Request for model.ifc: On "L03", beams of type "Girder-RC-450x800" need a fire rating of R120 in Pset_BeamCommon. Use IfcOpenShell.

First a look at what the model holds.

```python
import ifcopenshell
import ifcopenshell.util.element

model = ifcopenshell.open("model.ifc")
print(model.schema)
storey = next(s for s in model.by_type("IfcBuildingStorey") if s.Name == "L03")
beams = [e for e in ifcopenshell.util.element.get_decomposition(storey) if e.is_a("IfcBeam")]
seen = {}
for e in beams:
    element_type = ifcopenshell.util.element.get_type(e)
    key = (element_type.Name if element_type != e and element_type else None, ifcopenshell.util.element.get_pset(e, "Pset_BeamCommon", "FireRating"))
    seen[key] = seen.get(key, 0) + 1
for (name, value), count in sorted(seen.items(), key=str):
    print(count, "x", name, "|", value)
```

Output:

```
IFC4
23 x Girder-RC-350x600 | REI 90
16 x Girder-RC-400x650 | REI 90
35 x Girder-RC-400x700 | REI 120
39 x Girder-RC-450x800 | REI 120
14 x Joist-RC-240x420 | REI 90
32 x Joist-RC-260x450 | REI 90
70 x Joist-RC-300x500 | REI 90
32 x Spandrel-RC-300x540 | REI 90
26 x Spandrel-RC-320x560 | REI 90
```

```python
import ifcopenshell
import ifcopenshell.api.pset
import ifcopenshell.util.element

model = ifcopenshell.open("model.ifc")

storey = next(s for s in model.by_type("IfcBuildingStorey") if s.Name == "L03")
beams = [e for e in ifcopenshell.util.element.get_decomposition(storey) if e.is_a("IfcBeam")]

count = 0
for e in beams:
    element_type = ifcopenshell.util.element.get_type(e)
    if element_type in (None, e) or element_type.Name != "Girder-RC-450x800":
        continue
    # add_pset returns the element's existing set when there is one.
    pset = ifcopenshell.api.pset.add_pset(model, product=e, name="Pset_BeamCommon")
    ifcopenshell.api.pset.edit_pset(model, pset=pset, properties={"FireRating": "R120"})
    count += 1

print(count, "beams updated")

model.write("model_updated.ifc")
```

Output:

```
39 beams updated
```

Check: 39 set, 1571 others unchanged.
